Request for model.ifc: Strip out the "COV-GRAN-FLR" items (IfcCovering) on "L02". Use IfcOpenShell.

First a look at what the model holds.

```python
import ifcopenshell
import ifcopenshell.util.element

model = ifcopenshell.open("model.ifc")
print(model.schema)
storey = next(s for s in model.by_type("IfcBuildingStorey") if s.Name == "L02")
coverings = [e for e in ifcopenshell.util.element.get_decomposition(storey) if e.is_a("IfcCovering")]
seen = {}
for e in coverings:
    element_type = ifcopenshell.util.element.get_type(e)
    name = element_type.Name if element_type not in (None, e) else None
    seen[name] = seen.get(name, 0) + 1
for name, count in sorted(seen.items(), key=str):
    print(count, "x", name)
```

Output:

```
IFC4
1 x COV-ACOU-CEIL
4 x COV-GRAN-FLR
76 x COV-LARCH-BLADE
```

```python
import ifcopenshell
import ifcopenshell.api.root
import ifcopenshell.util.element

model = ifcopenshell.open("model.ifc")

storey = next(s for s in model.by_type("IfcBuildingStorey") if s.Name == "L02")
coverings = [e for e in ifcopenshell.util.element.get_decomposition(storey) if e.is_a("IfcCovering")]
targets = [e for e in coverings if (t := ifcopenshell.util.element.get_type(e)) not in (None, e) and t.Name == "COV-GRAN-FLR"]

for e in targets:
    ifcopenshell.api.root.remove_product(model, product=e)
print(len(targets), "removed")

model.write("model_updated.ifc")
```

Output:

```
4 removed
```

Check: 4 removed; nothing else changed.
